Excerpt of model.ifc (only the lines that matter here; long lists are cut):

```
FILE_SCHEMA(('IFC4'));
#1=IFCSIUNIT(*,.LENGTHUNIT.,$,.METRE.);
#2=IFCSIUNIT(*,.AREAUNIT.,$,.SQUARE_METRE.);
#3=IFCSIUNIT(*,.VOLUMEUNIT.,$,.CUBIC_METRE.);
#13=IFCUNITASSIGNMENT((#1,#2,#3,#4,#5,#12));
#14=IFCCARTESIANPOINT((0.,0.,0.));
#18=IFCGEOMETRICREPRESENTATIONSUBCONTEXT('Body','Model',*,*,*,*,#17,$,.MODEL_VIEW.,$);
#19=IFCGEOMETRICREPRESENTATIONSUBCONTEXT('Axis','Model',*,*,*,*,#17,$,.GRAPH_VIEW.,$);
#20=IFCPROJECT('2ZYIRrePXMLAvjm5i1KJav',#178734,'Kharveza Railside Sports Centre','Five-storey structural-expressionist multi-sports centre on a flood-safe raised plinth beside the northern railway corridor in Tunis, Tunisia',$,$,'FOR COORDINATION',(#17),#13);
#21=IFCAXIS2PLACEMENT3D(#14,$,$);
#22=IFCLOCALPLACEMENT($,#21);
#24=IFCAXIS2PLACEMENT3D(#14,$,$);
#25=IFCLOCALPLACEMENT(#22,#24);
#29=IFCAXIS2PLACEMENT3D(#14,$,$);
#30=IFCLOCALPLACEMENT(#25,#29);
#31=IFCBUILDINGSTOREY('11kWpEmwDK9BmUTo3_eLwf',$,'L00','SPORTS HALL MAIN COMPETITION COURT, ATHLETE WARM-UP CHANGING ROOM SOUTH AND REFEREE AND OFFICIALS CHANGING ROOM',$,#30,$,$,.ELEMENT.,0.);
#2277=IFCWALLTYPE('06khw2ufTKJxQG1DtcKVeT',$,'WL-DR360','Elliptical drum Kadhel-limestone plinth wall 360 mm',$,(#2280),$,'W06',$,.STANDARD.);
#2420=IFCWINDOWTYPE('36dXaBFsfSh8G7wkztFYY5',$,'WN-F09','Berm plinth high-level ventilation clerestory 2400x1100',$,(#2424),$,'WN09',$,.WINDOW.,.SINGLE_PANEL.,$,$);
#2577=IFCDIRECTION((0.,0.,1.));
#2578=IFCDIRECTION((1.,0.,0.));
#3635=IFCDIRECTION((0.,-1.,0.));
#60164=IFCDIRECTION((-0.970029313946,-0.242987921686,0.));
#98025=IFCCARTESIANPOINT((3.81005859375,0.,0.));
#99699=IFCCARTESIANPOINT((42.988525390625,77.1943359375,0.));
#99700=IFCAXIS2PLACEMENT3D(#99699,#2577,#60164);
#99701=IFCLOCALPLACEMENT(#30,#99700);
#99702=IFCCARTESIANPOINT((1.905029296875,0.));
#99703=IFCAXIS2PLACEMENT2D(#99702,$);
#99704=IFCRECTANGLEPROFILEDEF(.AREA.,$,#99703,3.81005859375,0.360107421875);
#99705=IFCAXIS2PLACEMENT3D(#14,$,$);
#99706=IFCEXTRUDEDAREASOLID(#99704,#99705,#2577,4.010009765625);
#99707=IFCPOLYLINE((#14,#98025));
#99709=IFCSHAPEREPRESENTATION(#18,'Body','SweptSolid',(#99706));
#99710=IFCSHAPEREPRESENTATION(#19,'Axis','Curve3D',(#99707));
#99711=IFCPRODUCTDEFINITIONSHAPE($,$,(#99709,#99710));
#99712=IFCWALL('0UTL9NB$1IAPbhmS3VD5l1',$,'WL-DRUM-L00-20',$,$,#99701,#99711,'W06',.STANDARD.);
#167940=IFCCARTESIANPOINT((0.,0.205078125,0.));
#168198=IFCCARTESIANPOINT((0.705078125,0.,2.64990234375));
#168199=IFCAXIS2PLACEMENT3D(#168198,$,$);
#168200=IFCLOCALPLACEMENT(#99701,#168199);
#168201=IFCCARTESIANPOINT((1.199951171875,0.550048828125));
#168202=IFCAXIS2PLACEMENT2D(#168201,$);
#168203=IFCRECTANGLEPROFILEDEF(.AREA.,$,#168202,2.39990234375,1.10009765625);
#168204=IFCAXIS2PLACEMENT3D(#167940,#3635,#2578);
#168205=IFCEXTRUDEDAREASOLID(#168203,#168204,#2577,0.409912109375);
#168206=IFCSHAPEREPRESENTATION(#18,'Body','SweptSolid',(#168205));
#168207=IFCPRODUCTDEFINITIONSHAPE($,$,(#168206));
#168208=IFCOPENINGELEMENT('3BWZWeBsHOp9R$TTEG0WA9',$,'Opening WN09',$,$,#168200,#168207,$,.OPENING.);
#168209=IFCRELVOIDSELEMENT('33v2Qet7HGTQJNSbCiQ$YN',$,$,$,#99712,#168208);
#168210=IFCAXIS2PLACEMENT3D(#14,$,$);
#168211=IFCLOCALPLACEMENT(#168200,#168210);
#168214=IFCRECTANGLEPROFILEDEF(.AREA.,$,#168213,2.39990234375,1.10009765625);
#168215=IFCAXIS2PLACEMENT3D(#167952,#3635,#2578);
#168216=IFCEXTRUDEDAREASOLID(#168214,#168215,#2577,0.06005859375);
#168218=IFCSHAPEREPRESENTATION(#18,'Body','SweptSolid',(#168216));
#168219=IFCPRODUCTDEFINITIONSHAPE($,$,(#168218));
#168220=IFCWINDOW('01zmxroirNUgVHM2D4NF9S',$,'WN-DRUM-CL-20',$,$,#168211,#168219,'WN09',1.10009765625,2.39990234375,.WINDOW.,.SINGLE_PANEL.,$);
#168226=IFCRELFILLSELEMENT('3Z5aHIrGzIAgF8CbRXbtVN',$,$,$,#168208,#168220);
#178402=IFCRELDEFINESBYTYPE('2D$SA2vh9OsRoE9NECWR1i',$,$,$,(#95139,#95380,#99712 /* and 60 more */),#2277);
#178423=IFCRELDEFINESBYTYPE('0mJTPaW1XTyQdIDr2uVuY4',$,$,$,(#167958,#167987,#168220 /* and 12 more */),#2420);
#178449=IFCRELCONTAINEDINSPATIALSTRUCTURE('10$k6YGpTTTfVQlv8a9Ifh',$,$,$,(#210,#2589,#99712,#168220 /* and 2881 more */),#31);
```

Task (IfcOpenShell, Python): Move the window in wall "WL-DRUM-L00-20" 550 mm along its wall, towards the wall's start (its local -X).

```python
import ifcopenshell
import ifcopenshell.api.geometry
import ifcopenshell.util.placement
import ifcopenshell.util.unit

model = ifcopenshell.open("model.ifc")
unit_scale = ifcopenshell.util.unit.calculate_unit_scale(model)

window = model.by_id(168220)
opening = window.FillsVoids[0].RelatingOpeningElement
wall = opening.VoidsElements[0].RelatingBuildingElement

wall_matrix = ifcopenshell.util.placement.get_local_placement(wall.ObjectPlacement)
shift = wall_matrix[:3, 0] * -0.55 / unit_scale
before = ifcopenshell.util.placement.get_local_placement(window.ObjectPlacement)[:3, 3].copy()

# The window is placed relative to its opening, so it follows when the opening moves.
matrix = ifcopenshell.util.placement.get_local_placement(opening.ObjectPlacement)
matrix[:3, 3] += shift
ifcopenshell.api.geometry.edit_object_placement(
    model, product=opening, matrix=matrix, is_si=False, should_transform_children=True
)

after = ifcopenshell.util.placement.get_local_placement(window.ObjectPlacement)[:3, 3]
print("window moved by", (after - before).round(3) + 0.0)

model.write("model_edited.ifc")
```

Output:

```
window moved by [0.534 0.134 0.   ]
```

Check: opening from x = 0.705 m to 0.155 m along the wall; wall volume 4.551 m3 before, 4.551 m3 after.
